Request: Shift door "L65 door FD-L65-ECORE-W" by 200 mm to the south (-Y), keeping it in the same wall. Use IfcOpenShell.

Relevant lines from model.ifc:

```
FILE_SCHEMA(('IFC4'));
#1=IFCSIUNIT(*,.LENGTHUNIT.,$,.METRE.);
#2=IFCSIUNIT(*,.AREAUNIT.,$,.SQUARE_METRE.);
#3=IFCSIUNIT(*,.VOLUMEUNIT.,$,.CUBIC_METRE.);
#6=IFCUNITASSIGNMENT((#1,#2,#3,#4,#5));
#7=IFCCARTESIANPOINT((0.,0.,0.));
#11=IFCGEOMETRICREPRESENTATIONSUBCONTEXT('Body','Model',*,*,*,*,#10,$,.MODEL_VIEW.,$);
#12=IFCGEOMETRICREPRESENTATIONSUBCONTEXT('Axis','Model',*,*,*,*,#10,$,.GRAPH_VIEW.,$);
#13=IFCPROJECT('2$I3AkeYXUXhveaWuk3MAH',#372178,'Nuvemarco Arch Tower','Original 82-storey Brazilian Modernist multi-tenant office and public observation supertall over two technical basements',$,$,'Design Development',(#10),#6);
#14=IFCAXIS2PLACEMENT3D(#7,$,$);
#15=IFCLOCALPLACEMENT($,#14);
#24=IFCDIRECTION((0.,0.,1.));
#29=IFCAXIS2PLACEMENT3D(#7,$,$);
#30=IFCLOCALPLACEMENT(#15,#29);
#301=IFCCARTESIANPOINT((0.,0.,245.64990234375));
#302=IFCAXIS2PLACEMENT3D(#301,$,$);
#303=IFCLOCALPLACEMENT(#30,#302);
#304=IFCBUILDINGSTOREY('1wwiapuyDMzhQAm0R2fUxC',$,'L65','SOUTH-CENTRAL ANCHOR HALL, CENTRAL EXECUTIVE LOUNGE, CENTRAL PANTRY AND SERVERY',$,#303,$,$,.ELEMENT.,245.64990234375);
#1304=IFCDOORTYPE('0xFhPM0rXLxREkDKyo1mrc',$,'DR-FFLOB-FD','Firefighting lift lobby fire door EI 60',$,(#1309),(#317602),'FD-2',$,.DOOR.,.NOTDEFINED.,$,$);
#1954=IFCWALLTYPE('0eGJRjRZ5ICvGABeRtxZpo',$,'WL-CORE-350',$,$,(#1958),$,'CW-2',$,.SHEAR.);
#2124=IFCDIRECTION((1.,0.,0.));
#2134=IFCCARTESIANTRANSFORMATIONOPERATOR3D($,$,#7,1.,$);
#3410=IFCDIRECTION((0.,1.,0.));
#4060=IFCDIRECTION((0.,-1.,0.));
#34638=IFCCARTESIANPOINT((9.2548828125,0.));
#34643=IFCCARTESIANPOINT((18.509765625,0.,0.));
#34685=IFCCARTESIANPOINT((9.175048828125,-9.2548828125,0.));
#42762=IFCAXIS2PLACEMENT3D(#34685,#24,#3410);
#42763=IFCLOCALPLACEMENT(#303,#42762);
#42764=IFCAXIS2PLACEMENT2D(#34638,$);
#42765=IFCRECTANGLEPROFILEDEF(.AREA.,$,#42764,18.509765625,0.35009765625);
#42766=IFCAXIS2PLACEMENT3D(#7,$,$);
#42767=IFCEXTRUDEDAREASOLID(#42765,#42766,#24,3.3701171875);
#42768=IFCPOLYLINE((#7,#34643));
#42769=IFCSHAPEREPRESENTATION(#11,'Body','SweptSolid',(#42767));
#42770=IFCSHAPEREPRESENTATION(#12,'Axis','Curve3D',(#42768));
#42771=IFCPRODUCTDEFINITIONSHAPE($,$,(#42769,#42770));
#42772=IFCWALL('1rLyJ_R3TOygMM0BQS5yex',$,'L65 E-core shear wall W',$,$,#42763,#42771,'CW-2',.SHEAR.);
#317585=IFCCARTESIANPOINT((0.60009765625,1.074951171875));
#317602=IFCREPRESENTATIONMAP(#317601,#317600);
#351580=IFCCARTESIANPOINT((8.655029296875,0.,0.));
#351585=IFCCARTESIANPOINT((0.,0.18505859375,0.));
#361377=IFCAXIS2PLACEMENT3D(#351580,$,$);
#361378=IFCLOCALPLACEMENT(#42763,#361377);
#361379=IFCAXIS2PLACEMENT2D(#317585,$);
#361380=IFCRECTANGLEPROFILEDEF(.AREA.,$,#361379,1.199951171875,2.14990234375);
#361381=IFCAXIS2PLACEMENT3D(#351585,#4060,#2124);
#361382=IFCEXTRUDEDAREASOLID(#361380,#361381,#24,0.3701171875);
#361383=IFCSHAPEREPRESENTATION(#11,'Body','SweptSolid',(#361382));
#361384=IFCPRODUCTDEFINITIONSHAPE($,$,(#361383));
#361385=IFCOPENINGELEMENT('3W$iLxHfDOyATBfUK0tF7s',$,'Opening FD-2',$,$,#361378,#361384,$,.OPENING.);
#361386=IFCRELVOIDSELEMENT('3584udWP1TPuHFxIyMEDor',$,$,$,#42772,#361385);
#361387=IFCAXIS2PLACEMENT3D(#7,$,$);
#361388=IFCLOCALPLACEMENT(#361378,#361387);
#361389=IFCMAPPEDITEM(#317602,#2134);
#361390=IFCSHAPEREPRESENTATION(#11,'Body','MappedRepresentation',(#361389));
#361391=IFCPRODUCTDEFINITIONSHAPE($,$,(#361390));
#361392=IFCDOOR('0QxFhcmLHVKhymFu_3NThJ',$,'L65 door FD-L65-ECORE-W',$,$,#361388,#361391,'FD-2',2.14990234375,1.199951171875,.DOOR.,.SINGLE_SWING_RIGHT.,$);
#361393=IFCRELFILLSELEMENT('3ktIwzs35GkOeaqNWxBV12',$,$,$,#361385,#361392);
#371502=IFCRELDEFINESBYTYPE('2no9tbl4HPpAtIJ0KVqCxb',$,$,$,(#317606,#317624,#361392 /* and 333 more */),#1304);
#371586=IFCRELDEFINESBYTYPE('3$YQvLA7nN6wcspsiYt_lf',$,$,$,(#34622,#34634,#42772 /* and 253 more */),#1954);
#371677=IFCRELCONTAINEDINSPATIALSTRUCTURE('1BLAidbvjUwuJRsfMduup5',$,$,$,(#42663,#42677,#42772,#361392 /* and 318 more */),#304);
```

```python
import ifcopenshell
import ifcopenshell.api.geometry
import ifcopenshell.util.placement
import ifcopenshell.util.unit

model = ifcopenshell.open("model.ifc")
unit_scale = ifcopenshell.util.unit.calculate_unit_scale(model)

door = model.by_guid("0QxFhcmLHVKhymFu_3NThJ")
opening = door.FillsVoids[0].RelatingOpeningElement
wall = opening.VoidsElements[0].RelatingBuildingElement

wall_matrix = ifcopenshell.util.placement.get_local_placement(wall.ObjectPlacement)
shift = wall_matrix[:3, 0] * -0.2 / unit_scale
before = ifcopenshell.util.placement.get_local_placement(door.ObjectPlacement)[:3, 3].copy()

# The door is placed relative to its opening, so it follows when the opening moves.
matrix = ifcopenshell.util.placement.get_local_placement(opening.ObjectPlacement)
matrix[:3, 3] += shift
ifcopenshell.api.geometry.edit_object_placement(
    model, product=opening, matrix=matrix, is_si=False, should_transform_children=True
)

after = ifcopenshell.util.placement.get_local_placement(door.ObjectPlacement)[:3, 3]
print("door moved by", (after - before).round(3) + 0.0)

model.write("model_rev.ifc")
```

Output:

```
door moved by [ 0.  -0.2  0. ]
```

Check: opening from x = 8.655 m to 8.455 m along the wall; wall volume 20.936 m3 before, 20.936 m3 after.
